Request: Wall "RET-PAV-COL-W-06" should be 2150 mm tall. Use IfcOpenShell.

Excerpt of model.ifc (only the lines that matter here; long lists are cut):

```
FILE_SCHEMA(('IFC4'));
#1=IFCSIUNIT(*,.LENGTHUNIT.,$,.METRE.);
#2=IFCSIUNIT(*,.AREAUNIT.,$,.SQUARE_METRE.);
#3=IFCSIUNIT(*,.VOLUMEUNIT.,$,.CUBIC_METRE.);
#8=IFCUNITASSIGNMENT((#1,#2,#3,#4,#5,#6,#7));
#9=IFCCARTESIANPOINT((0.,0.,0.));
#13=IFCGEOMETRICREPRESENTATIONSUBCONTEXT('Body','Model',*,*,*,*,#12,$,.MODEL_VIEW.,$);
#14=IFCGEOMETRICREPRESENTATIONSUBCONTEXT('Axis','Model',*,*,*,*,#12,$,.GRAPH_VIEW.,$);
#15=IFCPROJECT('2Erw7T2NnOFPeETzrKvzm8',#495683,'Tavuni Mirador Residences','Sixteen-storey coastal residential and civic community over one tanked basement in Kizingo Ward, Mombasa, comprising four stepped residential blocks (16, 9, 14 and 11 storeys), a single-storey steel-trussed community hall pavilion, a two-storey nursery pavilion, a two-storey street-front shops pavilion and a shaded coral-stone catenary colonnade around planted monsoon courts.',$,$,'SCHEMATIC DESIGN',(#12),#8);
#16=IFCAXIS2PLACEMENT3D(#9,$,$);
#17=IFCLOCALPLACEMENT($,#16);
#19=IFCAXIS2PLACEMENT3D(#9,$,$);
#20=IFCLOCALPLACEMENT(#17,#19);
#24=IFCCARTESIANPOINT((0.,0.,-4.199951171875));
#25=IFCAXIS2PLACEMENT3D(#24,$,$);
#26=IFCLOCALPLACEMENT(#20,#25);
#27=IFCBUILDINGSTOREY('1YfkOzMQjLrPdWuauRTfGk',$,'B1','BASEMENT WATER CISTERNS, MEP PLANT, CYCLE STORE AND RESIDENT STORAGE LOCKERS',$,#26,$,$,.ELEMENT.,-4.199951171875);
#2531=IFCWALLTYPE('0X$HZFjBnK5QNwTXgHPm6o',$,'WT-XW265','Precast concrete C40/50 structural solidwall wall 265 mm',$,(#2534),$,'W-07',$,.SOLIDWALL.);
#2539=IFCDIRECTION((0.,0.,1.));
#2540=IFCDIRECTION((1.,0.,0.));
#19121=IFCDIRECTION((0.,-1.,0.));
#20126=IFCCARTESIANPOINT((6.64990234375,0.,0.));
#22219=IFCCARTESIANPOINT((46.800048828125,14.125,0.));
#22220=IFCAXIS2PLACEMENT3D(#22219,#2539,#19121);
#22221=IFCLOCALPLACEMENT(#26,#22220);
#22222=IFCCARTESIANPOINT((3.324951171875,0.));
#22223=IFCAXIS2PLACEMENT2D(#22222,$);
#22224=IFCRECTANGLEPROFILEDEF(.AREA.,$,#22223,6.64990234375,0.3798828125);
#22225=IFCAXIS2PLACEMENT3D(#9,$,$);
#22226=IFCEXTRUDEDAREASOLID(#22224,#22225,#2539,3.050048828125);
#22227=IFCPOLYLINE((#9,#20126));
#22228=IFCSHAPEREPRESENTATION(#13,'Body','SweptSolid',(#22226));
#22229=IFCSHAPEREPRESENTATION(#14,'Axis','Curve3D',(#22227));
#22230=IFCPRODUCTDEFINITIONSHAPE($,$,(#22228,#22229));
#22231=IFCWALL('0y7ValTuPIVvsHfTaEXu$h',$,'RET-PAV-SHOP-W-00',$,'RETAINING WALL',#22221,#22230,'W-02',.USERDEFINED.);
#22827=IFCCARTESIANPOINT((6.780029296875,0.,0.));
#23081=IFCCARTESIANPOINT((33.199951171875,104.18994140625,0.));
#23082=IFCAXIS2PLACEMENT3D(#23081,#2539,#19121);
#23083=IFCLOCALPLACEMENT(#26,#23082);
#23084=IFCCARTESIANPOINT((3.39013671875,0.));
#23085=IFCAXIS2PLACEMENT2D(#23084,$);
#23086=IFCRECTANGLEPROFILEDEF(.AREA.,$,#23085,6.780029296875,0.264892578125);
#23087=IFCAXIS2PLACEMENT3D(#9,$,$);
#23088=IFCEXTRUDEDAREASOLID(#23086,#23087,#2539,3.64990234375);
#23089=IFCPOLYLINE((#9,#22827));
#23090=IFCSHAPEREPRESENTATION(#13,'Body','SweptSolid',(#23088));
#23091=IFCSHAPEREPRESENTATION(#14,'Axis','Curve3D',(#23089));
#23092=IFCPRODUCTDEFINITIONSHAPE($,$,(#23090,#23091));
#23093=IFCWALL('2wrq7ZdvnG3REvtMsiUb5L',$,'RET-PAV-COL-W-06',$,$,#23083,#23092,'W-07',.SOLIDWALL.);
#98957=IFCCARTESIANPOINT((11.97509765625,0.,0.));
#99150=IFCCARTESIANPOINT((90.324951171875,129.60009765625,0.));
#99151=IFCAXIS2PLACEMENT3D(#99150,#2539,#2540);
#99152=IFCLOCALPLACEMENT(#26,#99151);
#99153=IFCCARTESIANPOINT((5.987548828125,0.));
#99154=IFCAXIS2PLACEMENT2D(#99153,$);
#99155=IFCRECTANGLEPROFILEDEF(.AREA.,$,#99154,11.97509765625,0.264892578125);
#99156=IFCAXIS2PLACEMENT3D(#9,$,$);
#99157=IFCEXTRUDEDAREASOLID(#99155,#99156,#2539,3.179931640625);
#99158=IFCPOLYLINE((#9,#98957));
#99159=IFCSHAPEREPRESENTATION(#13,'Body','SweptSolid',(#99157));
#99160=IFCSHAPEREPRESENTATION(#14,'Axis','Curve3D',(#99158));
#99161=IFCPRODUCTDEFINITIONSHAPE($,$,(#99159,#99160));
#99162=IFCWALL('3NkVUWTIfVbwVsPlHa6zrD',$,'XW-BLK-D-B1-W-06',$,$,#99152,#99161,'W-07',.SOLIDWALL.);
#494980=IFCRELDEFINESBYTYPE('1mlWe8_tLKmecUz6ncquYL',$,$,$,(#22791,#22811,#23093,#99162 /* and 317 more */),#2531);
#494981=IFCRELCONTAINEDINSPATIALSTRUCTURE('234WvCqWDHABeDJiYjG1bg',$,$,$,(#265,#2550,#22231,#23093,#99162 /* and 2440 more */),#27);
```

```python
import ifcopenshell
import ifcopenshell.geom
import ifcopenshell.util.representation
import ifcopenshell.util.shape
import ifcopenshell.util.unit

model = ifcopenshell.open("model.ifc")
unit_scale = ifcopenshell.util.unit.calculate_unit_scale(model)
settings = ifcopenshell.geom.settings()


def volume(element):
    """Net volume in cubic metres, openings subtracted."""
    shape = ifcopenshell.geom.create_shape(settings, element)
    return ifcopenshell.util.shape.get_volume(shape.geometry)


wall = model.by_id(23093)
before = volume(wall)

body = ifcopenshell.util.representation.get_representation(wall, "Model", "Body")
solid = body.Items[0]
old_height = solid.Depth
solid.Depth = 2.15 / unit_scale
after = volume(wall)

print(f"height {old_height:g} -> {solid.Depth:g}, volume {before:.3f} -> {after:.3f} m3")

model.write("model_edited.ifc")
```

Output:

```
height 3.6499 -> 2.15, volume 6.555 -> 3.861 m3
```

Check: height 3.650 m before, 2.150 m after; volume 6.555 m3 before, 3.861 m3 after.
